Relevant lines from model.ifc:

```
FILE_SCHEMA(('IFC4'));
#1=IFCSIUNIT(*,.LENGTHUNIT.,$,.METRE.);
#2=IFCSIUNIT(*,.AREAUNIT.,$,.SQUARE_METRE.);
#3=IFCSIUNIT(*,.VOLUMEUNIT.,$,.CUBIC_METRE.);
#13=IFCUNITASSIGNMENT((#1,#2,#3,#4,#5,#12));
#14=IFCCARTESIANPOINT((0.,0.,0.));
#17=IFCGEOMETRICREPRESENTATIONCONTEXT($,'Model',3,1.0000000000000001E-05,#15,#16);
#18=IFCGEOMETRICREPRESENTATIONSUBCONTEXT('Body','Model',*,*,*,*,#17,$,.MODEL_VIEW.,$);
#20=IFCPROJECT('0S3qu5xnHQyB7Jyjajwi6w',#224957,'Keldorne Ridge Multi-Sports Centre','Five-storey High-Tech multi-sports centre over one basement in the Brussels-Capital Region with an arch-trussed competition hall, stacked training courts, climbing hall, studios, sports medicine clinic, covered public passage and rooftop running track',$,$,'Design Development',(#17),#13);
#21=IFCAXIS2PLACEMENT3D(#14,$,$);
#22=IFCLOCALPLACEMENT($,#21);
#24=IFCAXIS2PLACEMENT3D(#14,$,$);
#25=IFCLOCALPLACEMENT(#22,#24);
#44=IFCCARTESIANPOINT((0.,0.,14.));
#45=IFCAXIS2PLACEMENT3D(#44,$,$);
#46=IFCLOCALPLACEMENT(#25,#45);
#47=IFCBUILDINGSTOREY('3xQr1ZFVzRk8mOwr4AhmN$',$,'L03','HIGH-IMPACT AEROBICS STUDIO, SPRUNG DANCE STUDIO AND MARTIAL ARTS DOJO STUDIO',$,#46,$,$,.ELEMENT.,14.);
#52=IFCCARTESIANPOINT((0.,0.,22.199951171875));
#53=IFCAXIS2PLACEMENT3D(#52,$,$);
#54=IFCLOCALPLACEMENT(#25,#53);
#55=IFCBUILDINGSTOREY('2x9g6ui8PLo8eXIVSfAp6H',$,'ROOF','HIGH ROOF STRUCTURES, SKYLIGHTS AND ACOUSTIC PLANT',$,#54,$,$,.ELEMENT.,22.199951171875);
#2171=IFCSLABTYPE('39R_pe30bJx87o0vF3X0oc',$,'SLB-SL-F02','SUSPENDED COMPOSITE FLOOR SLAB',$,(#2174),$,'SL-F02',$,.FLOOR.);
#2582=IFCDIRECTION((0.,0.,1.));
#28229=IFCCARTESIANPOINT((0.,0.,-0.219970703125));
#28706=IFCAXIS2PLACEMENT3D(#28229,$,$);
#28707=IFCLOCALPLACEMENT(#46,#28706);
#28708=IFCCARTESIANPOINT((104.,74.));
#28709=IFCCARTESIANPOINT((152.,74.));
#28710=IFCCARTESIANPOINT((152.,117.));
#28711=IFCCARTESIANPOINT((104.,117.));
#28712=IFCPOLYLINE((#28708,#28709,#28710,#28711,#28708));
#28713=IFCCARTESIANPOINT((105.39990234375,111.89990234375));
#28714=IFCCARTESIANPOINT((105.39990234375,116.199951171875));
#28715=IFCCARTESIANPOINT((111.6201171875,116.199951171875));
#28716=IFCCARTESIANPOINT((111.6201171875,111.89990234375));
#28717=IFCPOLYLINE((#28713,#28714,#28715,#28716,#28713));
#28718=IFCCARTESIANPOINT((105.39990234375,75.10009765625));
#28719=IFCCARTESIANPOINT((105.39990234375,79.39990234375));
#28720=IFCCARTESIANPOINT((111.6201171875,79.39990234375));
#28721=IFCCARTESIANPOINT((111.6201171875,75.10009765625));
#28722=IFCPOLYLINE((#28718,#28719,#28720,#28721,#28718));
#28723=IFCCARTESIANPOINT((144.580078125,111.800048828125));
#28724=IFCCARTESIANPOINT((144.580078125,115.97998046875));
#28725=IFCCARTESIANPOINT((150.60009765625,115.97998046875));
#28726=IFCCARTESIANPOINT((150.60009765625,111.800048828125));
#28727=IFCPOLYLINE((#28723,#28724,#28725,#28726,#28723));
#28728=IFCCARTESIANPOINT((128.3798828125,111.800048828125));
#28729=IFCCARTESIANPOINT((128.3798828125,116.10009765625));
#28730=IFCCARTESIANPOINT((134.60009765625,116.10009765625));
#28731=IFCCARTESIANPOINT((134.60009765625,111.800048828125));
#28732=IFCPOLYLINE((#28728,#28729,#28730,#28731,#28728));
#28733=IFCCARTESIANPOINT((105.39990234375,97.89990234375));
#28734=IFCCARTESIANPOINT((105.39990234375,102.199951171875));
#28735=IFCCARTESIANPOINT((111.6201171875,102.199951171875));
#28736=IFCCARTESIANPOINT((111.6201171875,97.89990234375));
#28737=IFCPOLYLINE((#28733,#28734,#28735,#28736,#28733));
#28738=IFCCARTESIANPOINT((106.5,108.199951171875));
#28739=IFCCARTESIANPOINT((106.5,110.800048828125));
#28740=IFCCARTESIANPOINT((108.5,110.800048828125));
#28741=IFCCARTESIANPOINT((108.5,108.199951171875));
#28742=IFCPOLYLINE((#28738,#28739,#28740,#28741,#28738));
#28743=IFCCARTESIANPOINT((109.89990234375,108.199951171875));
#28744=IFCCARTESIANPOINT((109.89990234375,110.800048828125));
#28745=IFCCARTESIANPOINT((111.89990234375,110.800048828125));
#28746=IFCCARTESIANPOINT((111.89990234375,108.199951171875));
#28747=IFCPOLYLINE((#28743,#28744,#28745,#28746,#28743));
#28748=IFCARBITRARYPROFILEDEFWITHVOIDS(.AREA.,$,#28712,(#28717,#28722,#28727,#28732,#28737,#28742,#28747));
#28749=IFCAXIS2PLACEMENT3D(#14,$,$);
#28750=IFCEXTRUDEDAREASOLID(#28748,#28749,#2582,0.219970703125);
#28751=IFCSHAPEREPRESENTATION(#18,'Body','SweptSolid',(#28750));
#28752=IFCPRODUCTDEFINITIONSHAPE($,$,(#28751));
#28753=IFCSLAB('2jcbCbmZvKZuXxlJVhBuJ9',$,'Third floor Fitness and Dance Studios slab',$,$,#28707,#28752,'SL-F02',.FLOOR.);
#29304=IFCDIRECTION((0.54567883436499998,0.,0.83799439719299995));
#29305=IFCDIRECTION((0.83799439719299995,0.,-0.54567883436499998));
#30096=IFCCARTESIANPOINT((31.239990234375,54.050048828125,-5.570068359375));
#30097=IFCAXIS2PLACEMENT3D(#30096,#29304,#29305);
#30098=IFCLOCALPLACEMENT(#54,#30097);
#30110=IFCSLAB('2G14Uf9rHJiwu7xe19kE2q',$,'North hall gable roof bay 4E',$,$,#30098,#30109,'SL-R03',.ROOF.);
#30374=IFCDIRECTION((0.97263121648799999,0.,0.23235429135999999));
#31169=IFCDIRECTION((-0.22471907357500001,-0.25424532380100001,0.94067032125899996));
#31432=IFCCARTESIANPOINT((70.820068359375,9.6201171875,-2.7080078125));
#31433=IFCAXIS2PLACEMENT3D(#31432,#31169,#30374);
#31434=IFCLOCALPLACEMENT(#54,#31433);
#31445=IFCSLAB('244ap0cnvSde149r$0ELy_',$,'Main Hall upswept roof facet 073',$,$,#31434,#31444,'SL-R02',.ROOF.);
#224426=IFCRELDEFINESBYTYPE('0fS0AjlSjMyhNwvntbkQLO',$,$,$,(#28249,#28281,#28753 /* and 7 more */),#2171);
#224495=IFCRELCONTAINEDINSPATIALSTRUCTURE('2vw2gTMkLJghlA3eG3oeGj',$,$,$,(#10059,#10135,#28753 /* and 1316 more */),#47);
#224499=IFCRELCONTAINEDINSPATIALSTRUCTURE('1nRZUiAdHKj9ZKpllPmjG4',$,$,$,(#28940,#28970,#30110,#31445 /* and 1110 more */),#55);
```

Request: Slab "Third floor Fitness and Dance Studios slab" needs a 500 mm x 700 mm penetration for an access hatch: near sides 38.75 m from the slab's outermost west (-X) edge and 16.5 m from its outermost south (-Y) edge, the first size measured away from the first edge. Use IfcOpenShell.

```python
import numpy as np
import ifcopenshell
import ifcopenshell.api.feature
import ifcopenshell.api.geometry
import ifcopenshell.api.root
import ifcopenshell.geom
import ifcopenshell.util.placement
import ifcopenshell.util.representation
import ifcopenshell.util.shape
import ifcopenshell.util.unit

model = ifcopenshell.open("model.ifc")
unit_scale = ifcopenshell.util.unit.calculate_unit_scale(model)
settings = ifcopenshell.geom.settings()


def volume(element):
    """Net volume in cubic metres, openings subtracted."""
    shape = ifcopenshell.geom.create_shape(settings, element)
    return ifcopenshell.util.shape.get_volume(shape.geometry)


slab = model.by_guid("2jcbCbmZvKZuXxlJVhBuJ9")
before = volume(slab)

# Extent in the slab's own axes, in metres. The edges named are its -X and -Y sides.
slab_shape = ifcopenshell.geom.create_shape(settings, slab)
vertices = ifcopenshell.util.shape.get_vertices(slab_shape.geometry)
x_min, y_min, bottom = vertices.min(axis=0)
top = vertices[:, 2].max()

opening = ifcopenshell.api.root.create_entity(model, ifc_class="IfcOpeningElement", name="Access hatch opening", predefined_type="OPENING")
context = ifcopenshell.util.representation.get_context(model, "Model", "Body", "MODEL_VIEW")
width, depth = 0.5, 0.7
outline = [(0.0, 0.0), (width, 0.0), (width, depth), (0.0, depth), (0.0, 0.0)]
# Overshoot both faces by 50 mm so the cut is clean.
shape = ifcopenshell.api.geometry.add_slab_representation(
    model, context=context, depth=top - bottom + 0.1, polyline=outline
)
ifcopenshell.api.geometry.assign_representation(model, product=opening, representation=shape)

matrix = ifcopenshell.util.placement.get_local_placement(slab.ObjectPlacement)
matrix[:, 3] = matrix @ np.append(np.array([x_min + 38.75, y_min + 16.5, bottom - 0.05]) / unit_scale, 1.0)
ifcopenshell.api.geometry.edit_object_placement(model, product=opening, matrix=matrix, is_si=False)
ifcopenshell.api.feature.add_feature(model, feature=opening, element=slab)

after = volume(slab)

print(f"slab volume {before:.3f} -> {after:.3f} m3")

model.write("model_edited.ifc")
```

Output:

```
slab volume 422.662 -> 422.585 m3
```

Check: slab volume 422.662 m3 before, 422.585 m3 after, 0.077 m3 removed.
